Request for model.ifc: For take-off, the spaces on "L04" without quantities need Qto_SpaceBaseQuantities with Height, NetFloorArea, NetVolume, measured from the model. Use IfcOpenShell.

First a look at what the model holds.

```python
import ifcopenshell
import ifcopenshell.util.element
import ifcopenshell.util.unit

model = ifcopenshell.open("model.ifc")
print(model.schema)
for unit_type in ("LENGTHUNIT", "AREAUNIT", "VOLUMEUNIT"):
    print(unit_type, ifcopenshell.util.unit.calculate_unit_scale(model, unit_type))
storey = next(s for s in model.by_type("IfcBuildingStorey") if s.Name == "L04")
spaces = [e for e in ifcopenshell.util.element.get_decomposition(storey) if e.is_a("IfcSpace")]
for e in sorted(spaces, key=lambda e: e.id()):
    print(e.id(), e.is_a(), e.Name, list(ifcopenshell.util.element.get_psets(e, qtos_only=True)), sep=" | ")
```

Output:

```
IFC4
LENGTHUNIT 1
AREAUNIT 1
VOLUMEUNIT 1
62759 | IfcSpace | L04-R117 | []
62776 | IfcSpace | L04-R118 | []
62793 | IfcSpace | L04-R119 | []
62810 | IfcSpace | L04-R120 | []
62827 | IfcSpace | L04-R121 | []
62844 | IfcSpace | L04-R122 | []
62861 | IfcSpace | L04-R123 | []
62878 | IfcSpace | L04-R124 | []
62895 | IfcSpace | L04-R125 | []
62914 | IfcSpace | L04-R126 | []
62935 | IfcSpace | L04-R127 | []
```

```python
import ifcopenshell
import ifcopenshell.api.pset
import ifcopenshell.geom
import ifcopenshell.util.element
import ifcopenshell.util.shape
import ifcopenshell.util.unit

model = ifcopenshell.open("model.ifc")
unit_scale = ifcopenshell.util.unit.calculate_unit_scale(model)
area_scale = ifcopenshell.util.unit.calculate_unit_scale(model, "AREAUNIT")
volume_scale = ifcopenshell.util.unit.calculate_unit_scale(model, "VOLUMEUNIT")
settings = ifcopenshell.geom.settings()

storey = next(s for s in model.by_type("IfcBuildingStorey") if s.Name == "L04")
spaces = [e for e in ifcopenshell.util.element.get_decomposition(storey) if e.is_a("IfcSpace")]

for e in sorted(spaces, key=lambda e: e.id()):
    if ifcopenshell.util.element.get_psets(e, qtos_only=True, should_inherit=False):
        continue
    # Geometry comes back in metres, in the element's own axes.
    shape = ifcopenshell.geom.create_shape(settings, e)
    values = {
        "Height": ifcopenshell.util.shape.get_z(shape.geometry) / unit_scale,
        "NetFloorArea": ifcopenshell.util.shape.get_footprint_area(shape.geometry) / area_scale,
        "NetVolume": ifcopenshell.util.shape.get_volume(shape.geometry) / volume_scale,
    }
    qto = ifcopenshell.api.pset.add_qto(model, product=e, name="Qto_SpaceBaseQuantities")
    ifcopenshell.api.pset.edit_qto(model, qto=qto, properties=values)
    print(e.id(), {k: round(v, 3) for k, v in values.items()})

model.write("model_v2.ifc")
```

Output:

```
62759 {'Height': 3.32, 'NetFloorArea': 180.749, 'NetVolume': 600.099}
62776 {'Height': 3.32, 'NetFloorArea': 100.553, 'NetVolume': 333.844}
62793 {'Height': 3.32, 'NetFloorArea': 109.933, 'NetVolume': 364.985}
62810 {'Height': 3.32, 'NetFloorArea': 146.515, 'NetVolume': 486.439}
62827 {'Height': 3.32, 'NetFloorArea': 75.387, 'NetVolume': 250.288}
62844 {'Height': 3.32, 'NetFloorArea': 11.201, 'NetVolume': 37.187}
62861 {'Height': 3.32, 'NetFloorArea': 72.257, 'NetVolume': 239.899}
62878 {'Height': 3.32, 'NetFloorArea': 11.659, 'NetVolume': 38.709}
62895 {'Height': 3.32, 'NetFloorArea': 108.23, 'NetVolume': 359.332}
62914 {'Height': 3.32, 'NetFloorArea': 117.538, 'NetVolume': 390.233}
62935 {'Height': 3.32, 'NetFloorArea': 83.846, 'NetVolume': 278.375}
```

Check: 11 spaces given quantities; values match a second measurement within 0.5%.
